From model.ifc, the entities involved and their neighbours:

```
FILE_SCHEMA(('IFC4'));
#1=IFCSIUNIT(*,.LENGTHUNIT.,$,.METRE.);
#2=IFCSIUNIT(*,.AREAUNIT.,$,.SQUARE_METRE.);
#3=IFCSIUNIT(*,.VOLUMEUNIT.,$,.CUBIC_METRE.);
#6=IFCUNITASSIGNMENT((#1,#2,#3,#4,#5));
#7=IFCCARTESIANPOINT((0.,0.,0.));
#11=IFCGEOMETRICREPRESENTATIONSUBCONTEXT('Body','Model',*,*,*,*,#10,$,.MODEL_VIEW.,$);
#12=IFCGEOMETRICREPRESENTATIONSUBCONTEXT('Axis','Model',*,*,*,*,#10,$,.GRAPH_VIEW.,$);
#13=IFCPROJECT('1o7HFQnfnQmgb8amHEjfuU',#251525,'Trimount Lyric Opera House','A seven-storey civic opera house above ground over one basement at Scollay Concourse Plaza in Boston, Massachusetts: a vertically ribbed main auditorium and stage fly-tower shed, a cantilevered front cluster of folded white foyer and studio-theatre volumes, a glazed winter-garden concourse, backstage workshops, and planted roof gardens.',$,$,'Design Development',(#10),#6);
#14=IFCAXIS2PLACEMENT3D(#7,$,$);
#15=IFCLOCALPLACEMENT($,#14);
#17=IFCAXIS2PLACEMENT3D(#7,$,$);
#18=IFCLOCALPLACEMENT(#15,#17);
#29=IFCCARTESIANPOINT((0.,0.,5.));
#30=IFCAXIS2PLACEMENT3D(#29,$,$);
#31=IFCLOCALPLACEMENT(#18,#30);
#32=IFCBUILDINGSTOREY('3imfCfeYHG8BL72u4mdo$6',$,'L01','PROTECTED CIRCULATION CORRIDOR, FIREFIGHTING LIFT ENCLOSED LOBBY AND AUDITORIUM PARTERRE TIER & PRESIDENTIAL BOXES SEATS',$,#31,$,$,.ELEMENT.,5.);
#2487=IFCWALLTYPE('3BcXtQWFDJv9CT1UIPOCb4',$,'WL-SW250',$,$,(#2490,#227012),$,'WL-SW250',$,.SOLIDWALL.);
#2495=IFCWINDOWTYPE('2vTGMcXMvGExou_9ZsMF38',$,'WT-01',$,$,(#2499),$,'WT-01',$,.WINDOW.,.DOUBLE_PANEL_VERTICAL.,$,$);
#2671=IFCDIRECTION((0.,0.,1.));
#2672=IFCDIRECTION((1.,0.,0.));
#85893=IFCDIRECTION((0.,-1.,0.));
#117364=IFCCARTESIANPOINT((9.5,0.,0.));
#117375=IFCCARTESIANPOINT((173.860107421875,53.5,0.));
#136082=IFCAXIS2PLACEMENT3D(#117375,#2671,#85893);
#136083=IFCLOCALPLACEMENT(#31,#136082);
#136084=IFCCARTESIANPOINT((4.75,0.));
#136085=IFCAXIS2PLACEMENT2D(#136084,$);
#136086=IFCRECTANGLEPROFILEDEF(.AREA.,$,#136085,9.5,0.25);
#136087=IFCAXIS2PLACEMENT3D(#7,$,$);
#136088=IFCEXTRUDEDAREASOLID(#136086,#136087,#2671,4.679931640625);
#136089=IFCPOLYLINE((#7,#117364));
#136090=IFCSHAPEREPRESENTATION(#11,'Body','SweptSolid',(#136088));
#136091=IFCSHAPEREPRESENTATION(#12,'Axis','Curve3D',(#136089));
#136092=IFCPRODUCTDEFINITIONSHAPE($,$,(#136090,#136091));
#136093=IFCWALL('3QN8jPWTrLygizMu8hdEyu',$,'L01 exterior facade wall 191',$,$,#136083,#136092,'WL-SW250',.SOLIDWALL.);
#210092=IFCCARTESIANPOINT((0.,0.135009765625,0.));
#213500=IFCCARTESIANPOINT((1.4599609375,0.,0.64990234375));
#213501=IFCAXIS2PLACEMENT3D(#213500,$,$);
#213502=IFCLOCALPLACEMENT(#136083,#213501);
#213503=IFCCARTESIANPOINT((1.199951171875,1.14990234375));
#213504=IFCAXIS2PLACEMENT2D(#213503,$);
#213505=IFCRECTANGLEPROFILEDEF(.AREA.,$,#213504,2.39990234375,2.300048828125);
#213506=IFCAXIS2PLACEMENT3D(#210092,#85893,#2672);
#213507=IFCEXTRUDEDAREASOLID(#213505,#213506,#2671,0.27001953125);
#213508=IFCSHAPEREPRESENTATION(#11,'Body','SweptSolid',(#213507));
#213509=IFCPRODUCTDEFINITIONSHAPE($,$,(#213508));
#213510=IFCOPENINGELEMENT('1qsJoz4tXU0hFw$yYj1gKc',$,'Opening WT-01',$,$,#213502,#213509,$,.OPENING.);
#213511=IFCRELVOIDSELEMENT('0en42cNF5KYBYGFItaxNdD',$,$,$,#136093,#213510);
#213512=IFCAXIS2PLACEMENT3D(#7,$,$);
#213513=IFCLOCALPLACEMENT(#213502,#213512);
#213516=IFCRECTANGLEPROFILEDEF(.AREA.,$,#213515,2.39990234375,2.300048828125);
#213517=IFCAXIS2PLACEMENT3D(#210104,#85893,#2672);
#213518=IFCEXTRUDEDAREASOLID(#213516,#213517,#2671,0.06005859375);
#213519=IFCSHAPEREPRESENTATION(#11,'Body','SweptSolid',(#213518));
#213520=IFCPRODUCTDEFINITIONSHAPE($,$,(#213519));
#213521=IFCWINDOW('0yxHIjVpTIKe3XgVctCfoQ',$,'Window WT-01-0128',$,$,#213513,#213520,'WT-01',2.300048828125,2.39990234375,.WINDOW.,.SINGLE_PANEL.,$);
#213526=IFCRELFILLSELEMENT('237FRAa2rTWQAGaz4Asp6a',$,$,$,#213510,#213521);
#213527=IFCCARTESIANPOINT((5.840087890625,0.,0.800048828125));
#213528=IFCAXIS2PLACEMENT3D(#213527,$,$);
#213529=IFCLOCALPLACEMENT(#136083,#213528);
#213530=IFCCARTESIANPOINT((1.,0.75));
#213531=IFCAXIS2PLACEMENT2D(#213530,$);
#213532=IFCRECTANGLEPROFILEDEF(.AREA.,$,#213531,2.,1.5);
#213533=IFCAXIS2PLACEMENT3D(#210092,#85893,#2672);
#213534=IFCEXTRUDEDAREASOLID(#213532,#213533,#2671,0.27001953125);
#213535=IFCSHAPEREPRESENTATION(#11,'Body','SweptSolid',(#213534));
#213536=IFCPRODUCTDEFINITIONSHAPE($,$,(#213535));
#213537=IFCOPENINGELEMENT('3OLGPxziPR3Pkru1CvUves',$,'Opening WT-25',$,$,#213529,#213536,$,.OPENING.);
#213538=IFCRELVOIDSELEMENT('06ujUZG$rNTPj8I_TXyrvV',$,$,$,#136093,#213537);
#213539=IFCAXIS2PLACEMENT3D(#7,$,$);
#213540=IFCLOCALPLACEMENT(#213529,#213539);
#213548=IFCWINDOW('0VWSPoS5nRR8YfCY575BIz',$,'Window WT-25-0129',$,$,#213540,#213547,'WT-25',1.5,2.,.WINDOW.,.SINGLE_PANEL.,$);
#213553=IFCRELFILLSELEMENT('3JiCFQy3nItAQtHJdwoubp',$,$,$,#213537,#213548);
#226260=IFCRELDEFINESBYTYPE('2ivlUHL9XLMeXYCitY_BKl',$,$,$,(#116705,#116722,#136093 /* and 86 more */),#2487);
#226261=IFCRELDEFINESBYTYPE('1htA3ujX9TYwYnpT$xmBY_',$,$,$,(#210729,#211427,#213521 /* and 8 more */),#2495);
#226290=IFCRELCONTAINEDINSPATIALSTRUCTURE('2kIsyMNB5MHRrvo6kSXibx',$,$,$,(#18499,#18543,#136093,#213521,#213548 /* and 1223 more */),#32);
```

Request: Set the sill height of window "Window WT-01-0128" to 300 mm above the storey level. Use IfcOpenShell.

```python
import numpy as np
import ifcopenshell
import ifcopenshell.api.geometry
import ifcopenshell.geom
import ifcopenshell.util.element
import ifcopenshell.util.placement
import ifcopenshell.util.shape
import ifcopenshell.util.unit

model = ifcopenshell.open("model.ifc")
unit_scale = ifcopenshell.util.unit.calculate_unit_scale(model)

window = model.by_guid("0yxHIjVpTIKe3XgVctCfoQ")
opening = window.FillsVoids[0].RelatingOpeningElement
storey = ifcopenshell.util.element.get_container(window, ifc_class="IfcBuildingStorey")
level = ifcopenshell.util.placement.get_local_placement(storey.ObjectPlacement)[2, 3]

# The opening's origin need not be at the sill, so measure its lowest point.
shape = ifcopenshell.geom.create_shape(ifcopenshell.geom.settings(), opening)
bottom = ifcopenshell.util.shape.get_shape_bottom_elevation(shape, shape.geometry) / unit_scale
dz = level + 0.3 - bottom

shift = np.array([0.0, 0.0, dz])
# The window is placed relative to its opening, so it follows when the opening moves.
matrix = ifcopenshell.util.placement.get_local_placement(opening.ObjectPlacement)
matrix[:3, 3] += shift
ifcopenshell.api.geometry.edit_object_placement(
    model, product=opening, matrix=matrix, is_si=False, should_transform_children=True
)

print(f"moved by {dz * unit_scale:+.3f} m")

model.write("model-out.ifc")
```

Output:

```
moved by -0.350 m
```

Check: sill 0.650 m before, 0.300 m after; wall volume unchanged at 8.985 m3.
